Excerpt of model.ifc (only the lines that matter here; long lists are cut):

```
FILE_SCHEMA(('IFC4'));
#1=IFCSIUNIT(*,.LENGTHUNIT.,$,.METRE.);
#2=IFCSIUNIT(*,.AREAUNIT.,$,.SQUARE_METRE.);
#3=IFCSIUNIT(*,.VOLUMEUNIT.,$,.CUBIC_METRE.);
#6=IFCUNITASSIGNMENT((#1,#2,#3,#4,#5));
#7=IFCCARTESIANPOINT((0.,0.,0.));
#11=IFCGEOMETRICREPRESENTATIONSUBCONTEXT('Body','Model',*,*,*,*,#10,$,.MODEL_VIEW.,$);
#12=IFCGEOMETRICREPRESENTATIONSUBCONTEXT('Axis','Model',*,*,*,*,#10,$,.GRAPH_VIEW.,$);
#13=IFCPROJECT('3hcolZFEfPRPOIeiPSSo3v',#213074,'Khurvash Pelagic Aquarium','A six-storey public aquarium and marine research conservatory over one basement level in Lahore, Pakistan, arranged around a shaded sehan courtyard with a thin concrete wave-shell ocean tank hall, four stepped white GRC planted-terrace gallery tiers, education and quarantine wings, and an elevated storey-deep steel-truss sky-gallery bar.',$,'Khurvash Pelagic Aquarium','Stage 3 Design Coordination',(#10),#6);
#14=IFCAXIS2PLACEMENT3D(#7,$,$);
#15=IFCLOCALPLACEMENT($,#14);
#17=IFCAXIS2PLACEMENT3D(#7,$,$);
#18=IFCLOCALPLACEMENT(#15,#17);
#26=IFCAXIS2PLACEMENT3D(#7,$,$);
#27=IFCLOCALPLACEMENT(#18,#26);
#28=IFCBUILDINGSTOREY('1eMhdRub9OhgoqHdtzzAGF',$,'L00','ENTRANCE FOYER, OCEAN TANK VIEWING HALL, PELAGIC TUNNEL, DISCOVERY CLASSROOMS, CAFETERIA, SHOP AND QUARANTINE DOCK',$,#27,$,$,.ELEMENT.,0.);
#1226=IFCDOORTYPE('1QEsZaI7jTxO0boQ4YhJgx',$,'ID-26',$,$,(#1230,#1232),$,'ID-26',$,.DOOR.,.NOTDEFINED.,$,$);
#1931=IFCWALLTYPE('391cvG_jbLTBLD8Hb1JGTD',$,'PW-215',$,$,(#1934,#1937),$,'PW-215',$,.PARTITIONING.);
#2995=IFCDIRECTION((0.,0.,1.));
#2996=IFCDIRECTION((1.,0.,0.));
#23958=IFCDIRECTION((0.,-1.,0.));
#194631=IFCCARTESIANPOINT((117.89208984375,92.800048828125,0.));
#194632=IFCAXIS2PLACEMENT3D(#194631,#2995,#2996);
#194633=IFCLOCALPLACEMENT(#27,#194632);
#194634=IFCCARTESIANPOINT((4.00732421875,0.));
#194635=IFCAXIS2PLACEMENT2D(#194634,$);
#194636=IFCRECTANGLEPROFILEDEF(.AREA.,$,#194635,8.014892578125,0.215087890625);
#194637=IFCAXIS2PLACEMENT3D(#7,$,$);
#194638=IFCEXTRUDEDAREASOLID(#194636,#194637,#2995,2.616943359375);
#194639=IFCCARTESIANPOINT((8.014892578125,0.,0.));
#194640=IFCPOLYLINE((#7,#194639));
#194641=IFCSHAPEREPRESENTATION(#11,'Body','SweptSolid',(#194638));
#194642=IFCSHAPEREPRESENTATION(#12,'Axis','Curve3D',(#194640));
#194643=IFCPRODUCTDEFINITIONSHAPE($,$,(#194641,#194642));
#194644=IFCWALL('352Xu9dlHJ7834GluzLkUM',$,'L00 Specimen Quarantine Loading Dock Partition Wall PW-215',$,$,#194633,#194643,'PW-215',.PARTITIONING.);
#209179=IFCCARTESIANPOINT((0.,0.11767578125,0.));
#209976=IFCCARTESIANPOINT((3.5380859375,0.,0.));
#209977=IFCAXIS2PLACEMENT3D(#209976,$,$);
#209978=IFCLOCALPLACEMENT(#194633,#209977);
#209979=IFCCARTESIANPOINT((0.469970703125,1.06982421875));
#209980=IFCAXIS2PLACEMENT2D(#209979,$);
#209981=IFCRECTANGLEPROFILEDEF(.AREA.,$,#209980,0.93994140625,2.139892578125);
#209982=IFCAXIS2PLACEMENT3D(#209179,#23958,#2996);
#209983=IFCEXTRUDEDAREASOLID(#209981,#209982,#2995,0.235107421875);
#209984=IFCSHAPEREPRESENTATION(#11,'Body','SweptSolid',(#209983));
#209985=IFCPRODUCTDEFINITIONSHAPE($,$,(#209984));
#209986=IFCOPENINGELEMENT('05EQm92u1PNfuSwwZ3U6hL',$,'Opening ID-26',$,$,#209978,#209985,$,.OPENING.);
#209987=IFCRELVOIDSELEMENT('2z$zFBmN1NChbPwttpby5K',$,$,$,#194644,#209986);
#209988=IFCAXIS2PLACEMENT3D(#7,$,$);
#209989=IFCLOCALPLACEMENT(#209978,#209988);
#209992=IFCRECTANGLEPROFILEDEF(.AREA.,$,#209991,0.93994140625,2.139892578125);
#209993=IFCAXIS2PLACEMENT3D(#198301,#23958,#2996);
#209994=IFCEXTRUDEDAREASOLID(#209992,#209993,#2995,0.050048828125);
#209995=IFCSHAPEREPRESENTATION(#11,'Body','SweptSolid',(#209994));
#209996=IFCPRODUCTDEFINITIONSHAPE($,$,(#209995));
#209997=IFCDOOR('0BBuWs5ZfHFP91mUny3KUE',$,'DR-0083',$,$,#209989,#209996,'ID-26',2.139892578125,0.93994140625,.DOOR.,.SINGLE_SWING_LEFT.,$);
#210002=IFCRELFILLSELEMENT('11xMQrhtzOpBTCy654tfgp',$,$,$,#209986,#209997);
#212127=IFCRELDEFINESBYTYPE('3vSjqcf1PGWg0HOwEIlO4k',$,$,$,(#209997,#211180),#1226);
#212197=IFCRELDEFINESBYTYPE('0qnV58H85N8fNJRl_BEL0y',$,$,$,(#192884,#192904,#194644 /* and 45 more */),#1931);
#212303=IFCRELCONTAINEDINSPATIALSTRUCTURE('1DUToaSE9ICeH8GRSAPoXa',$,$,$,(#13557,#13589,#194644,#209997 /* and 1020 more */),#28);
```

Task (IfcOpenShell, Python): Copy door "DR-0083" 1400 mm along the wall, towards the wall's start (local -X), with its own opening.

```python
import ifcopenshell
import ifcopenshell.api.feature
import ifcopenshell.api.geometry
import ifcopenshell.api.root
import ifcopenshell.geom
import ifcopenshell.util.element
import ifcopenshell.util.placement
import ifcopenshell.util.shape
import ifcopenshell.util.unit

model = ifcopenshell.open("model.ifc")
unit_scale = ifcopenshell.util.unit.calculate_unit_scale(model)
settings = ifcopenshell.geom.settings()


def volume(element):
    """Net volume in cubic metres, openings subtracted."""
    shape = ifcopenshell.geom.create_shape(settings, element)
    return ifcopenshell.util.shape.get_volume(shape.geometry)


door = model.by_guid("0BBuWs5ZfHFP91mUny3KUE")
opening = door.FillsVoids[0].RelatingOpeningElement
wall = opening.VoidsElements[0].RelatingBuildingElement
before = volume(wall)
shift = ifcopenshell.util.placement.get_local_placement(wall.ObjectPlacement)[:3, 0] * -1.4 / unit_scale

# copy_class copies the void relationship, type, container and properties, but no geometry.
new_opening = ifcopenshell.api.root.copy_class(model, product=opening)
new_opening.Representation = ifcopenshell.util.element.copy_deep(
    model, opening.Representation, exclude=["IfcGeometricRepresentationContext", "IfcRepresentationMap"]
)
new_door = ifcopenshell.api.root.copy_class(model, product=door)
new_door.Representation = ifcopenshell.util.element.copy_deep(
    model, door.Representation, exclude=["IfcGeometricRepresentationContext", "IfcRepresentationMap"]
)
new_door.Tag = None
ifcopenshell.api.feature.add_filling(model, opening=new_opening, element=new_door)

for old, new in ((opening, new_opening), (door, new_door)):
    matrix = ifcopenshell.util.placement.get_local_placement(old.ObjectPlacement)
    matrix[:3, 3] += shift
    ifcopenshell.api.geometry.edit_object_placement(model, product=new, matrix=matrix, is_si=False)

after = volume(wall)

print(f"wall volume {before:.3f} -> {after:.3f} m3")

model.write("model-out.ifc")
```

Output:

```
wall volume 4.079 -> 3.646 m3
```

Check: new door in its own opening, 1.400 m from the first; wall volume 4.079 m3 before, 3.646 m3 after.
